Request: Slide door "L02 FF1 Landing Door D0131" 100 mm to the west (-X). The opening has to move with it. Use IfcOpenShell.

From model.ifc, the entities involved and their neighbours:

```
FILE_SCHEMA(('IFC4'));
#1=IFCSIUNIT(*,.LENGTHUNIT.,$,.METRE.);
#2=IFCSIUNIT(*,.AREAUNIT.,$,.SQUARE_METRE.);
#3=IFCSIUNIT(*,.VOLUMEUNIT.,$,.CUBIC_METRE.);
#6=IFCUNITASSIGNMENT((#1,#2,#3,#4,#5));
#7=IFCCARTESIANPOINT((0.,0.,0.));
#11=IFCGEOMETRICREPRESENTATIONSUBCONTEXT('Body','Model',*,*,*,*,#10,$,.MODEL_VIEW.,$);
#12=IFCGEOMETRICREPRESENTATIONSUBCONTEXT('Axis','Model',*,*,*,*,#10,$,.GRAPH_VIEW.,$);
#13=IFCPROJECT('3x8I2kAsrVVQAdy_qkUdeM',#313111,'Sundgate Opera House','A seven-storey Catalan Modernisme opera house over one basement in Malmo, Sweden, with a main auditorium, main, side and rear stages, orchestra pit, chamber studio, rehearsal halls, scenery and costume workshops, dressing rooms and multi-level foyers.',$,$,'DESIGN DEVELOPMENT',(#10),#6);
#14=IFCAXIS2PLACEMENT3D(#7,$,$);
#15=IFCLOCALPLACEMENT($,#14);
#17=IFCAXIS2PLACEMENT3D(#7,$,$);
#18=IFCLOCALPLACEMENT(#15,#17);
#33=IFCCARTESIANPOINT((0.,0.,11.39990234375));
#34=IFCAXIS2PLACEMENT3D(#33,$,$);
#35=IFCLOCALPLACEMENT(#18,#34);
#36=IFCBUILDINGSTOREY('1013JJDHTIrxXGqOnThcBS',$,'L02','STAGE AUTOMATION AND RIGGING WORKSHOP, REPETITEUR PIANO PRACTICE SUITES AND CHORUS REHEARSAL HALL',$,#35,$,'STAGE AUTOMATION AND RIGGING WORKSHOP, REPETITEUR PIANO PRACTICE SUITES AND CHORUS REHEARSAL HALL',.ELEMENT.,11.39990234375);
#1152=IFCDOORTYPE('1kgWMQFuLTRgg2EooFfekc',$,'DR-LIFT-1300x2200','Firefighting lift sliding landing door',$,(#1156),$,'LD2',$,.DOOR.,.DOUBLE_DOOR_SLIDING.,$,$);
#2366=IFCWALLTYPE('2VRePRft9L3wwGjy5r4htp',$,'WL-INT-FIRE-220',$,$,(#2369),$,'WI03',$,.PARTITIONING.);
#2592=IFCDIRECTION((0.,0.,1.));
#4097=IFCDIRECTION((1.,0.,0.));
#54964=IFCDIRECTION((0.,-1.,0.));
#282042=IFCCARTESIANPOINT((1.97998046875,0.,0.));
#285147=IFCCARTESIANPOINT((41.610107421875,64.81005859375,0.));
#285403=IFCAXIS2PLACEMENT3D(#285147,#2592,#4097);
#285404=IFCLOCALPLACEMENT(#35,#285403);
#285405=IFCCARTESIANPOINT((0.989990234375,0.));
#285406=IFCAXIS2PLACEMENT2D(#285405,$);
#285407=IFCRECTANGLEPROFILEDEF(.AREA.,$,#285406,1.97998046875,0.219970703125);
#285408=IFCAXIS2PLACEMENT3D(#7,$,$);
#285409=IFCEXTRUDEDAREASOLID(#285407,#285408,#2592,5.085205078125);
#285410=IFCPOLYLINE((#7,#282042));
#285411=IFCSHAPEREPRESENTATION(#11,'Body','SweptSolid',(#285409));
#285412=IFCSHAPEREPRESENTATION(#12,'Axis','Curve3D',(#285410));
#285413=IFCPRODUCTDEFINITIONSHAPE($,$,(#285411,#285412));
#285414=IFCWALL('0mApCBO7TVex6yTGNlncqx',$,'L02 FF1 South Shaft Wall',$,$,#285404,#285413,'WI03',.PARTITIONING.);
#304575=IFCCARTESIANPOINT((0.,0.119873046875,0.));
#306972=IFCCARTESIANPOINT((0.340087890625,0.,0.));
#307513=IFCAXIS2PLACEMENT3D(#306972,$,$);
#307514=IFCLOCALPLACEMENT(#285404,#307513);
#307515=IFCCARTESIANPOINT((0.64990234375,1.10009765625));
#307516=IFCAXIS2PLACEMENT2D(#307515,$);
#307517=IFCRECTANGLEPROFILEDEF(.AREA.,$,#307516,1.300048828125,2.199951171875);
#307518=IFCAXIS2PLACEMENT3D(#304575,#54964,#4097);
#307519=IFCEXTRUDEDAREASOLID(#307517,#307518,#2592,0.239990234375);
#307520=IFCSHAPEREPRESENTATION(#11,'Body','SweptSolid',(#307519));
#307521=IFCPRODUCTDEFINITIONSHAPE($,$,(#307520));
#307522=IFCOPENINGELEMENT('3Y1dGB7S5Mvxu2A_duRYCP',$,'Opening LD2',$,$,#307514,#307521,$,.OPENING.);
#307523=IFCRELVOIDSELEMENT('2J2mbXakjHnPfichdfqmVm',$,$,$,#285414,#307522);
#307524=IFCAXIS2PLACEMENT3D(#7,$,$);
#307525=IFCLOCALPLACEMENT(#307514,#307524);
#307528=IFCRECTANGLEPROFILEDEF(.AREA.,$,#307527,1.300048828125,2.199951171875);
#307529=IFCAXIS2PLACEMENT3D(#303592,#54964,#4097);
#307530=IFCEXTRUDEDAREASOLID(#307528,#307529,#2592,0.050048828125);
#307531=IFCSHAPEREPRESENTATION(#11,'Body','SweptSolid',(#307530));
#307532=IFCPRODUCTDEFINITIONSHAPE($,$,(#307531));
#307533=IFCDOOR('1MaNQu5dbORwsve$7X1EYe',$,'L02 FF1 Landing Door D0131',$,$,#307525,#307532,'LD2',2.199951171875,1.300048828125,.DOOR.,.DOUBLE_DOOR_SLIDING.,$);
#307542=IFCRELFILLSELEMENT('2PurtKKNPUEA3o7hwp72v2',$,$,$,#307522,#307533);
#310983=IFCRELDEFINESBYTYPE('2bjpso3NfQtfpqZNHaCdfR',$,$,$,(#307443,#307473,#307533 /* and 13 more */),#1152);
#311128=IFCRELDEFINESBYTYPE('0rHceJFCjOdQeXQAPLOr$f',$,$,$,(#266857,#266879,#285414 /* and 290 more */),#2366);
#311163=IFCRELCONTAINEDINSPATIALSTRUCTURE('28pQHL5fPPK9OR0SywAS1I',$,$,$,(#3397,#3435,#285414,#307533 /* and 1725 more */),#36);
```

```python
import ifcopenshell
import ifcopenshell.api.geometry
import ifcopenshell.util.placement

model = ifcopenshell.open("model.ifc")

door = model.by_guid("1MaNQu5dbORwsve$7X1EYe")
opening = door.FillsVoids[0].RelatingOpeningElement
wall = opening.VoidsElements[0].RelatingBuildingElement

wall_matrix = ifcopenshell.util.placement.get_local_placement(wall.ObjectPlacement)
shift = wall_matrix[:3, 0] * -0.1
before = ifcopenshell.util.placement.get_local_placement(door.ObjectPlacement)[:3, 3].copy()

# The door is placed relative to its opening, so it follows when the opening moves.
matrix = ifcopenshell.util.placement.get_local_placement(opening.ObjectPlacement)
matrix[:3, 3] += shift
ifcopenshell.api.geometry.edit_object_placement(
    model, product=opening, matrix=matrix, is_si=False, should_transform_children=True
)

after = ifcopenshell.util.placement.get_local_placement(door.ObjectPlacement)[:3, 3]
print("door moved by", (after - before).round(3) + 0.0)

model.write("model_v2.ifc")
```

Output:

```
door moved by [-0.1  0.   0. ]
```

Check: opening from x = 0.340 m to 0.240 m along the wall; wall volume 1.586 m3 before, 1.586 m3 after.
